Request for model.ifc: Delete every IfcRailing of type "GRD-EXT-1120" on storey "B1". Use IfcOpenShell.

First a look at what the model holds.

```python
import ifcopenshell
import ifcopenshell.util.element

model = ifcopenshell.open("model.ifc")
print(model.schema)
storey = next(s for s in model.by_type("IfcBuildingStorey") if s.Name == "B1")
railings = [e for e in ifcopenshell.util.element.get_decomposition(storey) if e.is_a("IfcRailing")]
seen = {}
for e in railings:
    element_type = ifcopenshell.util.element.get_type(e)
    name = element_type.Name if element_type not in (None, e) else None
    seen[name] = seen.get(name, 0) + 1
for name, count in sorted(seen.items(), key=str):
    print(count, "x", name)
```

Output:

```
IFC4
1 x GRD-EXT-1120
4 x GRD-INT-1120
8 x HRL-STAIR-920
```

```python
import ifcopenshell
import ifcopenshell.api.root
import ifcopenshell.util.element

model = ifcopenshell.open("model.ifc")

storey = next(s for s in model.by_type("IfcBuildingStorey") if s.Name == "B1")
railings = [e for e in ifcopenshell.util.element.get_decomposition(storey) if e.is_a("IfcRailing")]
targets = [e for e in railings if (t := ifcopenshell.util.element.get_type(e)) not in (None, e) and t.Name == "GRD-EXT-1120"]

for e in targets:
    ifcopenshell.api.root.remove_product(model, product=e)
print(len(targets), "removed")

model.write("model_updated.ifc")
```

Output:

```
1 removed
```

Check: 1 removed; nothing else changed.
